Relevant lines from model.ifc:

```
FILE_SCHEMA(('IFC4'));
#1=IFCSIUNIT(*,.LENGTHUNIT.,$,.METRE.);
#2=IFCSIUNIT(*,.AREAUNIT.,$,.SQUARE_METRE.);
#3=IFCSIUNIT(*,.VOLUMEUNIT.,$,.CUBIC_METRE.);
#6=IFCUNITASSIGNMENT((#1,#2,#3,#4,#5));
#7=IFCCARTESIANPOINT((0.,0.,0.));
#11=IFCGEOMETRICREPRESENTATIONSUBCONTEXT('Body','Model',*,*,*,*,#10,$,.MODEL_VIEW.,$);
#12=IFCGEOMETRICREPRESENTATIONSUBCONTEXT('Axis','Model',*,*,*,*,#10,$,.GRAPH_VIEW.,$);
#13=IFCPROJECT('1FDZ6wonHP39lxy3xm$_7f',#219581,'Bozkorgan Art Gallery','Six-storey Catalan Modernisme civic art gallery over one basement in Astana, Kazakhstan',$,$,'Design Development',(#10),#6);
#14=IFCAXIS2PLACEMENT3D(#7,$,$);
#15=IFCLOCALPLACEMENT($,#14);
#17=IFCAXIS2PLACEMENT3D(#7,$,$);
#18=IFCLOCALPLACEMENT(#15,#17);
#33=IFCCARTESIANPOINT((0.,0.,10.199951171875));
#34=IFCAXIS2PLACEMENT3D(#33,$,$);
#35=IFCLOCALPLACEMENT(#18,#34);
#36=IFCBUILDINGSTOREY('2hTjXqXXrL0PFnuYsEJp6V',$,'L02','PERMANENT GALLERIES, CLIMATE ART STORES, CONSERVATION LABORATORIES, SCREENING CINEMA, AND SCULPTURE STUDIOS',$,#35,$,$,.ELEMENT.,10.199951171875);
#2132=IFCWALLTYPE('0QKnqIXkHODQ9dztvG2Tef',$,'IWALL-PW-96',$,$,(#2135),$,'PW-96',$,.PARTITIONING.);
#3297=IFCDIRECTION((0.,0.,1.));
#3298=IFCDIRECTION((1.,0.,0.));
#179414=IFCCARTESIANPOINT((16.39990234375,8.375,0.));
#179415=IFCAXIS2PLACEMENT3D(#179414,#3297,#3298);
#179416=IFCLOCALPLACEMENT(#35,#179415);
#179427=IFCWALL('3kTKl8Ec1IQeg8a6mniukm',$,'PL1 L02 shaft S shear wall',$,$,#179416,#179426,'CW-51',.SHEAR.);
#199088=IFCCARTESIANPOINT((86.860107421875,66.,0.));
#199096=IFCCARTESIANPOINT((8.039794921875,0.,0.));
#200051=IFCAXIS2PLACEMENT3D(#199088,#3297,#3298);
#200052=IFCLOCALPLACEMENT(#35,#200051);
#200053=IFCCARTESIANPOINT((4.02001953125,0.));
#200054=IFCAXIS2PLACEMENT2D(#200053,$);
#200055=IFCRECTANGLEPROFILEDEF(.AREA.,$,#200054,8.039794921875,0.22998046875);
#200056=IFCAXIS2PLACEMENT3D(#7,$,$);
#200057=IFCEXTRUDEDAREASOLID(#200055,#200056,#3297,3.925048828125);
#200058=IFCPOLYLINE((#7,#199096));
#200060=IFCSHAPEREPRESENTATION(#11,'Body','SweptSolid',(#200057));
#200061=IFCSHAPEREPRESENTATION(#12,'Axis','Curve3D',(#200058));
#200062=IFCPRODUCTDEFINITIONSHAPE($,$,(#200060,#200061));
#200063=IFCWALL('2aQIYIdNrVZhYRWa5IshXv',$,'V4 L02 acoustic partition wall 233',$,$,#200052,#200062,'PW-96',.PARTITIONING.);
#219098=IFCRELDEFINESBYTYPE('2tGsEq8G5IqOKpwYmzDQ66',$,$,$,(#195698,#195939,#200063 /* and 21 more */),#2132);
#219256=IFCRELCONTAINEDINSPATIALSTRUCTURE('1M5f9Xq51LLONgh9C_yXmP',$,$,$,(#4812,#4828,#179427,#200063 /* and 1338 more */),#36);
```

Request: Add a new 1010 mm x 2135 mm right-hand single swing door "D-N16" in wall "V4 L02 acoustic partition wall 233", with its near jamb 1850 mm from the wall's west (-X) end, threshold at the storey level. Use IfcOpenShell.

```python
import numpy as np
import ifcopenshell
import ifcopenshell.api.feature
import ifcopenshell.api.geometry
import ifcopenshell.api.root
import ifcopenshell.api.spatial
import ifcopenshell.geom
import ifcopenshell.util.element
import ifcopenshell.util.placement
import ifcopenshell.util.representation
import ifcopenshell.util.shape
import ifcopenshell.util.unit

model = ifcopenshell.open("model.ifc")
unit_scale = ifcopenshell.util.unit.calculate_unit_scale(model)
settings = ifcopenshell.geom.settings()


def volume(element):
    """Net volume in cubic metres, openings subtracted."""
    shape = ifcopenshell.geom.create_shape(settings, element)
    return ifcopenshell.util.shape.get_volume(shape.geometry)


wall = model.by_guid("2aQIYIdNrVZhYRWa5IshXv")
storey = ifcopenshell.util.element.get_container(wall, ifc_class="IfcBuildingStorey")
context = ifcopenshell.util.representation.get_context(model, "Model", "Body", "MODEL_VIEW")
before = volume(wall)

width, height, from_end, sill = 1.01, 2.135, 1.85, 0.0  # metres

# The wall runs along its own X axis, and the end named is its -X end.
wall_shape = ifcopenshell.geom.create_shape(settings, wall)
x, y, z = ifcopenshell.util.shape.get_vertices(wall_shape.geometry).T
start = x.min() + from_end
face, thickness = float(y.min()), float(y.max() - y.min())
wall_matrix = ifcopenshell.util.placement.get_local_placement(wall.ObjectPlacement)
level = ifcopenshell.util.placement.get_local_placement(storey.ObjectPlacement)[2, 3]


def in_wall(x, y):
    """Placement at x, y metres in the wall's axes, at sill height."""
    matrix = wall_matrix.copy()
    matrix[:, 3] = wall_matrix @ np.array([x / unit_scale, y / unit_scale, 0.0, 1.0])
    matrix[2, 3] = level + sill / unit_scale
    return matrix


# Opening: a box that overshoots both wall faces by 50 mm.
opening = ifcopenshell.api.root.create_entity(model, ifc_class="IfcOpeningElement", predefined_type="OPENING")
box = ifcopenshell.api.geometry.add_wall_representation(
    model, context=context, length=width, height=height, thickness=thickness + 0.1
)
ifcopenshell.api.geometry.assign_representation(model, product=opening, representation=box)
ifcopenshell.api.geometry.edit_object_placement(model, product=opening, matrix=in_wall(start, face - 0.05), is_si=False)
ifcopenshell.api.feature.add_feature(model, feature=opening, element=wall)

door = ifcopenshell.api.root.create_entity(model, ifc_class="IfcDoor", name="D-N16", predefined_type="DOOR")
door.OverallWidth, door.OverallHeight = width / unit_scale, height / unit_scale
door.OperationType = "SINGLE_SWING_RIGHT"
body = ifcopenshell.api.geometry.add_door_representation(
    model,
    context=context,
    overall_width=door.OverallWidth,
    overall_height=door.OverallHeight,
    operation_type="SINGLE_SWING_RIGHT",
    lining_properties={"LiningDepth": thickness / unit_scale, "ThresholdDepth": thickness / unit_scale},
)
ifcopenshell.api.geometry.assign_representation(model, product=door, representation=body)
ifcopenshell.api.spatial.assign_container(model, products=[door], relating_structure=storey)
ifcopenshell.api.feature.add_filling(model, opening=opening, element=door)

# The lining spans the wall, so the door starts at the wall face.
ifcopenshell.api.geometry.edit_object_placement(model, product=door, matrix=in_wall(start, face), is_si=False)

after = volume(wall)

print(f"wall volume {before:.3f} -> {after:.3f} m3")

model.write("model_rev.ifc")
```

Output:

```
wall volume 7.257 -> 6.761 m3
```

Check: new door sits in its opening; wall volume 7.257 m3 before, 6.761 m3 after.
